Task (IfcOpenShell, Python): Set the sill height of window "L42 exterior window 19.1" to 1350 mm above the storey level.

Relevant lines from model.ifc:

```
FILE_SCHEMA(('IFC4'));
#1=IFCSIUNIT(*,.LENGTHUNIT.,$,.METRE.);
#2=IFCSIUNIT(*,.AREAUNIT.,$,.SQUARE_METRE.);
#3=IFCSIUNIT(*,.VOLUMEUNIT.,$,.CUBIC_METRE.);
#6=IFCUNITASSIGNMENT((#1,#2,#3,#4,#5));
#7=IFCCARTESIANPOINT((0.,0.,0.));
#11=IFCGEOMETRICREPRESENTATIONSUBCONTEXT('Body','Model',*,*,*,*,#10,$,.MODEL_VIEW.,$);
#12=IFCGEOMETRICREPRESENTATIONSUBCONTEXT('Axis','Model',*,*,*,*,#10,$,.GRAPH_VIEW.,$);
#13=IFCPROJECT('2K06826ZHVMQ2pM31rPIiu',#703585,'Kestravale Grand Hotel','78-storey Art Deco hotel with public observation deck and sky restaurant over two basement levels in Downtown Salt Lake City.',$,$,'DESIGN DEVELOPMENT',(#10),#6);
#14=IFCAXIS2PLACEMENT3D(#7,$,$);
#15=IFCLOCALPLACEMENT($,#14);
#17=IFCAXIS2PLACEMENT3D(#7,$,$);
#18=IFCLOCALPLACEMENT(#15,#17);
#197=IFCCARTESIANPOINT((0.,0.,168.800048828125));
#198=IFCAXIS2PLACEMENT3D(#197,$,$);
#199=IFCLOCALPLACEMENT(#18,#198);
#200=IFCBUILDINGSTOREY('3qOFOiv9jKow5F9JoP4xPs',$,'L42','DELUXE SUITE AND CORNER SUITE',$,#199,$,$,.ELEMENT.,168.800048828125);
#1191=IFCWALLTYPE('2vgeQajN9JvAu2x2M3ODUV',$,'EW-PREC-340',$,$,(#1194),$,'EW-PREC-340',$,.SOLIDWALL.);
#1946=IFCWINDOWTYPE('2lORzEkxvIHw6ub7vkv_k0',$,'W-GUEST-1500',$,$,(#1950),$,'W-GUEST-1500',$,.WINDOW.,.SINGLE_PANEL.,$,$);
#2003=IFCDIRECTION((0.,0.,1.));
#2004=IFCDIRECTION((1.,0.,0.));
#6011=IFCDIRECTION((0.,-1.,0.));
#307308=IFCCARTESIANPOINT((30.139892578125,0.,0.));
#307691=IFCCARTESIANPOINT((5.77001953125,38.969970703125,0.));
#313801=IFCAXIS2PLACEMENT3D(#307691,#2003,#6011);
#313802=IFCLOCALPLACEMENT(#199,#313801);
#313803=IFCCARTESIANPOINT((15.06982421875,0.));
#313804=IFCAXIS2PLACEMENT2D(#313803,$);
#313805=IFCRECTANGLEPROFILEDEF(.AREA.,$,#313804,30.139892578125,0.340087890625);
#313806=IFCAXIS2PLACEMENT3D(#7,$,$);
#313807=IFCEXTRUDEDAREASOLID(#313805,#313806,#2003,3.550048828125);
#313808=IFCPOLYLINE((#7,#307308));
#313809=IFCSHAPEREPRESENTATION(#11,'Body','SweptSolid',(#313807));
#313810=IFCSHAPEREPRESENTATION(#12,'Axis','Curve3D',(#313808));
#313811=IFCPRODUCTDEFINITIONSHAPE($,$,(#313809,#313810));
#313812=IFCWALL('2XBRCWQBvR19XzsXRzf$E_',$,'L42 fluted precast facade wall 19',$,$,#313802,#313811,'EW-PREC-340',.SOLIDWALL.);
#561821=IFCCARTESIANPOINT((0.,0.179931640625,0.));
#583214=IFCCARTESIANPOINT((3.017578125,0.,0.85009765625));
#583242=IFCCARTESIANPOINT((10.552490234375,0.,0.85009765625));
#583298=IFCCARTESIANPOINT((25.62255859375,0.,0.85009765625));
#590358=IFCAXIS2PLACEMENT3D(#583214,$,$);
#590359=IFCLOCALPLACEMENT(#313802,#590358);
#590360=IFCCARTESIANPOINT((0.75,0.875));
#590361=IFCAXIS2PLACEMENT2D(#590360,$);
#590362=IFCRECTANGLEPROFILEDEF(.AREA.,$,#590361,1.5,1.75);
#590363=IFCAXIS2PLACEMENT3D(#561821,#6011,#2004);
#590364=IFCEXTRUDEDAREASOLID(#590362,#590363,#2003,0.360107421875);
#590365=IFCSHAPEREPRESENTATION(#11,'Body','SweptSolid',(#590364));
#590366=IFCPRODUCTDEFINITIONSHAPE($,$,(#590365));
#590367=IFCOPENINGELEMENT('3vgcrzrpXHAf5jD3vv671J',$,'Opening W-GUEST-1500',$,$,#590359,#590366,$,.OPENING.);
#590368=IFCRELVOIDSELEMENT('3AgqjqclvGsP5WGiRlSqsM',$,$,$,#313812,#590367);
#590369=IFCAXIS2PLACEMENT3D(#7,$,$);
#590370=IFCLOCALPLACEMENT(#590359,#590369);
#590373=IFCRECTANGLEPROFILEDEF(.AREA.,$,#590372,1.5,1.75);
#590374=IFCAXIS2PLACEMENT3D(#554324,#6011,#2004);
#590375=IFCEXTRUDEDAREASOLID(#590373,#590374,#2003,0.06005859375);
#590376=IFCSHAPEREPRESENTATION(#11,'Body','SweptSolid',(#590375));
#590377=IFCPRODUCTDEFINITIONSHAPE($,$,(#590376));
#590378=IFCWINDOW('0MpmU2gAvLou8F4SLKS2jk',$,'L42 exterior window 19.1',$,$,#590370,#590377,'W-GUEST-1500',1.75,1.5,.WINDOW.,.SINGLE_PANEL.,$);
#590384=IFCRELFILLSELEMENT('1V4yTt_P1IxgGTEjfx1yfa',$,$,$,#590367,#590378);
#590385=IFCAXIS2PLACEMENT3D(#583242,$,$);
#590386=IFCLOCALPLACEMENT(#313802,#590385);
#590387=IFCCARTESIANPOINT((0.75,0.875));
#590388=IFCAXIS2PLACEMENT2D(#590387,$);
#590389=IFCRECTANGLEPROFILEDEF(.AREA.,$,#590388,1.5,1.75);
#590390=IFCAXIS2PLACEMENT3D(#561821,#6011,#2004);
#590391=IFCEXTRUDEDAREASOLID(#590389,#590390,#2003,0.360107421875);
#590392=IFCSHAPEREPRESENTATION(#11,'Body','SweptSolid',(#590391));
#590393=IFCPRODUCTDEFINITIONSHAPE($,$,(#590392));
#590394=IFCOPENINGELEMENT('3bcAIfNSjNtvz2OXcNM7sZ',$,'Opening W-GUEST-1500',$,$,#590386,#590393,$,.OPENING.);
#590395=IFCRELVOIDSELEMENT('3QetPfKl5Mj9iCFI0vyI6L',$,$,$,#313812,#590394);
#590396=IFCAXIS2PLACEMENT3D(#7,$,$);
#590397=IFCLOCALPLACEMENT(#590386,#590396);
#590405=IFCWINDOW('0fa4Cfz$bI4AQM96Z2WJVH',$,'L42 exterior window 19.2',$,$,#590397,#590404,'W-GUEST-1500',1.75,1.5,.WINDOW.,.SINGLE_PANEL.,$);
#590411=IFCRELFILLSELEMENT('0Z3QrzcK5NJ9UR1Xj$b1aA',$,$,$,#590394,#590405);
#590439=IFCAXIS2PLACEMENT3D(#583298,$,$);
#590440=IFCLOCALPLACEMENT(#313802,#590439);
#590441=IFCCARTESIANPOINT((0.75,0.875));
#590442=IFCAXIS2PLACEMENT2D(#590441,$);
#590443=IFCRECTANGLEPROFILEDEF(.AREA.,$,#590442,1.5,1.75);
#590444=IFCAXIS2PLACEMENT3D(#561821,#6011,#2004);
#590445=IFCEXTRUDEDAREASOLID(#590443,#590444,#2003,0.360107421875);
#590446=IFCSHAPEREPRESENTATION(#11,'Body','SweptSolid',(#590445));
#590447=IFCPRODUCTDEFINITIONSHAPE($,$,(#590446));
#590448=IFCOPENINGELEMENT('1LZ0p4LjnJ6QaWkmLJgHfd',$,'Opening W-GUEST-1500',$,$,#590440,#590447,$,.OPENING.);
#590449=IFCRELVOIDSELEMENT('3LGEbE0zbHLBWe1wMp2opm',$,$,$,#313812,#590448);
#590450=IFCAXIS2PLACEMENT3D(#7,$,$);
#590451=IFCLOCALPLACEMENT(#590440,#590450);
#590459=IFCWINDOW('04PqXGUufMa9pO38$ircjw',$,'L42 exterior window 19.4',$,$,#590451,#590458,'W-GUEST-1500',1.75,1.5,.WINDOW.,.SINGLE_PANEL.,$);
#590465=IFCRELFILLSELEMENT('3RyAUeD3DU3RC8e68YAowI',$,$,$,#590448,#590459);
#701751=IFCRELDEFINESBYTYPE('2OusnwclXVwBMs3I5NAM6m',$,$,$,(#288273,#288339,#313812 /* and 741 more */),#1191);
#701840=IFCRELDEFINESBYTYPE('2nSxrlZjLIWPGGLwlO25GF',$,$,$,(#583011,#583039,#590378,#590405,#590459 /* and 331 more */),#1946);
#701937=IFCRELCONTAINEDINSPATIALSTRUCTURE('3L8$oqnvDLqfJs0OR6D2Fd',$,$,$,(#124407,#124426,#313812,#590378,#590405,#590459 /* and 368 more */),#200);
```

```python
import numpy as np
import ifcopenshell
import ifcopenshell.api.geometry
import ifcopenshell.geom
import ifcopenshell.util.element
import ifcopenshell.util.placement
import ifcopenshell.util.shape
import ifcopenshell.util.unit

model = ifcopenshell.open("model.ifc")
unit_scale = ifcopenshell.util.unit.calculate_unit_scale(model)

window = model.by_id(590378)
opening = window.FillsVoids[0].RelatingOpeningElement
storey = ifcopenshell.util.element.get_container(window, ifc_class="IfcBuildingStorey")
level = ifcopenshell.util.placement.get_local_placement(storey.ObjectPlacement)[2, 3]

# The opening's origin need not be at the sill, so measure its lowest point.
shape = ifcopenshell.geom.create_shape(ifcopenshell.geom.settings(), opening)
bottom = ifcopenshell.util.shape.get_shape_bottom_elevation(shape, shape.geometry) / unit_scale
dz = level + 1.35 - bottom

shift = np.array([0.0, 0.0, dz])
# The window is placed relative to its opening, so it follows when the opening moves.
matrix = ifcopenshell.util.placement.get_local_placement(opening.ObjectPlacement)
matrix[:3, 3] += shift
ifcopenshell.api.geometry.edit_object_placement(
    model, product=opening, matrix=matrix, is_si=False, should_transform_children=True
)

print(f"moved by {dz * unit_scale:+.3f} m")

model.write("model_edited.ifc")
```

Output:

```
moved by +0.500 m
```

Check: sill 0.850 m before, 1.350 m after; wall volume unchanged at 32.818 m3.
